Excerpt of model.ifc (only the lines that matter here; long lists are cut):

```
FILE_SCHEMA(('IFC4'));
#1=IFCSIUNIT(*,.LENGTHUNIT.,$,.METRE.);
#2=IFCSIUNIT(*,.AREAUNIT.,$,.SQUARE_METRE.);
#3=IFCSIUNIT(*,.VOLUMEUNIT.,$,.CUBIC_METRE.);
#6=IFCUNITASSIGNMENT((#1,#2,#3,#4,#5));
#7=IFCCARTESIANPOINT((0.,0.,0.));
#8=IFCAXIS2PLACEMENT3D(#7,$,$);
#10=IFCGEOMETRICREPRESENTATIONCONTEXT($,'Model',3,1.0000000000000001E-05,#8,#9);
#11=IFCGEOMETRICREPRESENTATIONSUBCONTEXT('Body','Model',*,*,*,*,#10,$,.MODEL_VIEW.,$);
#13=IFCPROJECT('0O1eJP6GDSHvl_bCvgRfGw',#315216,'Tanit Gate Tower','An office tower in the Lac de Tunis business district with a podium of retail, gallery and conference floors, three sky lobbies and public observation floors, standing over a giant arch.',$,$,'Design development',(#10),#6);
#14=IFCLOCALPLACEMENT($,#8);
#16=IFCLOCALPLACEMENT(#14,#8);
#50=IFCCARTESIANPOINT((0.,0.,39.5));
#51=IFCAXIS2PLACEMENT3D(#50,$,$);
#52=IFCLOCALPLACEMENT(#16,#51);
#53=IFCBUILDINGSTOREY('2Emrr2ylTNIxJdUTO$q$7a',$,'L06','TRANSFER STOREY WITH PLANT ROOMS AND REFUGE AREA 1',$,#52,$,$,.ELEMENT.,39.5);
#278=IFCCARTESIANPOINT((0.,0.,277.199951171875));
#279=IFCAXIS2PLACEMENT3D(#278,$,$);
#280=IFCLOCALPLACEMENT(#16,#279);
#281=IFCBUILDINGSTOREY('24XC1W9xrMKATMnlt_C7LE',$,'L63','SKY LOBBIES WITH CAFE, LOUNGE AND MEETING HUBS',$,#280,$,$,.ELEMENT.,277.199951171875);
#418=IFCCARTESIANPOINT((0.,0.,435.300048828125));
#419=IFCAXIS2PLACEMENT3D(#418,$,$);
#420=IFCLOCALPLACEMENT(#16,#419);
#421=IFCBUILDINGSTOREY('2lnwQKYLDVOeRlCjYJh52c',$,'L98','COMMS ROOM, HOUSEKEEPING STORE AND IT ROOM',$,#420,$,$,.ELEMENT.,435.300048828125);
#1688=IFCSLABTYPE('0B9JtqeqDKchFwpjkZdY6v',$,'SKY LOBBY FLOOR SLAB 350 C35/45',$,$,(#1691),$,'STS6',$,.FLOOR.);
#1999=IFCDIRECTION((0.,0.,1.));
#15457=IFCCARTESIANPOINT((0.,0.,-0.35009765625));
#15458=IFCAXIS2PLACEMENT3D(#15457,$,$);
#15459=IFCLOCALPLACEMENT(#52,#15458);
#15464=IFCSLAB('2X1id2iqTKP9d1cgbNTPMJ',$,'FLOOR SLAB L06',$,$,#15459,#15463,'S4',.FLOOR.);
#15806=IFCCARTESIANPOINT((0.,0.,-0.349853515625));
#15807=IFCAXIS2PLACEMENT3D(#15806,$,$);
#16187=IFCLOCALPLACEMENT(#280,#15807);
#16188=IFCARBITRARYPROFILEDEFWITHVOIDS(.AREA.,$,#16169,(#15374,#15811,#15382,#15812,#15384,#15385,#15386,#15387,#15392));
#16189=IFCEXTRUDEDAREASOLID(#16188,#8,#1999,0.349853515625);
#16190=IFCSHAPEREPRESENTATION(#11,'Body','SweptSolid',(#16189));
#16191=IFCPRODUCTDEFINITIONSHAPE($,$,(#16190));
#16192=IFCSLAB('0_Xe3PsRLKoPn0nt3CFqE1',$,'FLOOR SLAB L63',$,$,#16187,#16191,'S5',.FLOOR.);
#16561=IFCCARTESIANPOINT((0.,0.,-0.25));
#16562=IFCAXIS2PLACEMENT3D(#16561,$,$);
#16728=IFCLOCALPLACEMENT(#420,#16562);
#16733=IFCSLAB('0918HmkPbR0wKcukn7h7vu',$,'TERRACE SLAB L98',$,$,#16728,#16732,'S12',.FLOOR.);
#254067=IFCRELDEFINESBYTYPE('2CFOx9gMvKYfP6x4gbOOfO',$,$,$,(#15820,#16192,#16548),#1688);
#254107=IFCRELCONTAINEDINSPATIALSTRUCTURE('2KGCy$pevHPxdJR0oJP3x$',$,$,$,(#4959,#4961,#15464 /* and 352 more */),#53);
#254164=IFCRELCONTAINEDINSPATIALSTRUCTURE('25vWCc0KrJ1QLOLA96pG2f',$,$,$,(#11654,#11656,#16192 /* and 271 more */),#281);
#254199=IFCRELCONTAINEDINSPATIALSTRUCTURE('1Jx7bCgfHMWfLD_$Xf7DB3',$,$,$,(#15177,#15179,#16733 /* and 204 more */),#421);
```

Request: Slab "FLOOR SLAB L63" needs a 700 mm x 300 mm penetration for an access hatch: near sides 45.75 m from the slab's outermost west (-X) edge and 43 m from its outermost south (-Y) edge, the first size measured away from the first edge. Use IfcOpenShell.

```python
import numpy as np
import ifcopenshell
import ifcopenshell.api.feature
import ifcopenshell.api.geometry
import ifcopenshell.api.root
import ifcopenshell.geom
import ifcopenshell.util.placement
import ifcopenshell.util.representation
import ifcopenshell.util.shape
import ifcopenshell.util.unit

model = ifcopenshell.open("model.ifc")
unit_scale = ifcopenshell.util.unit.calculate_unit_scale(model)
settings = ifcopenshell.geom.settings()


def volume(element):
    """Net volume in cubic metres, openings subtracted."""
    shape = ifcopenshell.geom.create_shape(settings, element)
    return ifcopenshell.util.shape.get_volume(shape.geometry)


slab = model.by_guid("0_Xe3PsRLKoPn0nt3CFqE1")
before = volume(slab)

# Extent in the slab's own axes, in metres. The edges named are its -X and -Y sides.
slab_shape = ifcopenshell.geom.create_shape(settings, slab)
vertices = ifcopenshell.util.shape.get_vertices(slab_shape.geometry)
x_min, y_min, bottom = vertices.min(axis=0)
top = vertices[:, 2].max()

opening = ifcopenshell.api.root.create_entity(model, ifc_class="IfcOpeningElement", name="Access hatch opening", predefined_type="OPENING")
context = ifcopenshell.util.representation.get_context(model, "Model", "Body", "MODEL_VIEW")
width, depth = 0.7, 0.3
outline = [(0.0, 0.0), (width, 0.0), (width, depth), (0.0, depth), (0.0, 0.0)]
# Overshoot both faces by 50 mm so the cut is clean.
shape = ifcopenshell.api.geometry.add_slab_representation(
    model, context=context, depth=top - bottom + 0.1, polyline=outline
)
ifcopenshell.api.geometry.assign_representation(model, product=opening, representation=shape)

matrix = ifcopenshell.util.placement.get_local_placement(slab.ObjectPlacement)
matrix[:, 3] = matrix @ np.append(np.array([x_min + 45.75, y_min + 43, bottom - 0.05]) / unit_scale, 1.0)
ifcopenshell.api.geometry.edit_object_placement(model, product=opening, matrix=matrix, is_si=False)
ifcopenshell.api.feature.add_feature(model, feature=opening, element=slab)

after = volume(slab)

print(f"slab volume {before:.3f} -> {after:.3f} m3")

model.write("model_v2.ifc")
```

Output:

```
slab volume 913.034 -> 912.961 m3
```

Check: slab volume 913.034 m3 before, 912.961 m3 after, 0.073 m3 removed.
